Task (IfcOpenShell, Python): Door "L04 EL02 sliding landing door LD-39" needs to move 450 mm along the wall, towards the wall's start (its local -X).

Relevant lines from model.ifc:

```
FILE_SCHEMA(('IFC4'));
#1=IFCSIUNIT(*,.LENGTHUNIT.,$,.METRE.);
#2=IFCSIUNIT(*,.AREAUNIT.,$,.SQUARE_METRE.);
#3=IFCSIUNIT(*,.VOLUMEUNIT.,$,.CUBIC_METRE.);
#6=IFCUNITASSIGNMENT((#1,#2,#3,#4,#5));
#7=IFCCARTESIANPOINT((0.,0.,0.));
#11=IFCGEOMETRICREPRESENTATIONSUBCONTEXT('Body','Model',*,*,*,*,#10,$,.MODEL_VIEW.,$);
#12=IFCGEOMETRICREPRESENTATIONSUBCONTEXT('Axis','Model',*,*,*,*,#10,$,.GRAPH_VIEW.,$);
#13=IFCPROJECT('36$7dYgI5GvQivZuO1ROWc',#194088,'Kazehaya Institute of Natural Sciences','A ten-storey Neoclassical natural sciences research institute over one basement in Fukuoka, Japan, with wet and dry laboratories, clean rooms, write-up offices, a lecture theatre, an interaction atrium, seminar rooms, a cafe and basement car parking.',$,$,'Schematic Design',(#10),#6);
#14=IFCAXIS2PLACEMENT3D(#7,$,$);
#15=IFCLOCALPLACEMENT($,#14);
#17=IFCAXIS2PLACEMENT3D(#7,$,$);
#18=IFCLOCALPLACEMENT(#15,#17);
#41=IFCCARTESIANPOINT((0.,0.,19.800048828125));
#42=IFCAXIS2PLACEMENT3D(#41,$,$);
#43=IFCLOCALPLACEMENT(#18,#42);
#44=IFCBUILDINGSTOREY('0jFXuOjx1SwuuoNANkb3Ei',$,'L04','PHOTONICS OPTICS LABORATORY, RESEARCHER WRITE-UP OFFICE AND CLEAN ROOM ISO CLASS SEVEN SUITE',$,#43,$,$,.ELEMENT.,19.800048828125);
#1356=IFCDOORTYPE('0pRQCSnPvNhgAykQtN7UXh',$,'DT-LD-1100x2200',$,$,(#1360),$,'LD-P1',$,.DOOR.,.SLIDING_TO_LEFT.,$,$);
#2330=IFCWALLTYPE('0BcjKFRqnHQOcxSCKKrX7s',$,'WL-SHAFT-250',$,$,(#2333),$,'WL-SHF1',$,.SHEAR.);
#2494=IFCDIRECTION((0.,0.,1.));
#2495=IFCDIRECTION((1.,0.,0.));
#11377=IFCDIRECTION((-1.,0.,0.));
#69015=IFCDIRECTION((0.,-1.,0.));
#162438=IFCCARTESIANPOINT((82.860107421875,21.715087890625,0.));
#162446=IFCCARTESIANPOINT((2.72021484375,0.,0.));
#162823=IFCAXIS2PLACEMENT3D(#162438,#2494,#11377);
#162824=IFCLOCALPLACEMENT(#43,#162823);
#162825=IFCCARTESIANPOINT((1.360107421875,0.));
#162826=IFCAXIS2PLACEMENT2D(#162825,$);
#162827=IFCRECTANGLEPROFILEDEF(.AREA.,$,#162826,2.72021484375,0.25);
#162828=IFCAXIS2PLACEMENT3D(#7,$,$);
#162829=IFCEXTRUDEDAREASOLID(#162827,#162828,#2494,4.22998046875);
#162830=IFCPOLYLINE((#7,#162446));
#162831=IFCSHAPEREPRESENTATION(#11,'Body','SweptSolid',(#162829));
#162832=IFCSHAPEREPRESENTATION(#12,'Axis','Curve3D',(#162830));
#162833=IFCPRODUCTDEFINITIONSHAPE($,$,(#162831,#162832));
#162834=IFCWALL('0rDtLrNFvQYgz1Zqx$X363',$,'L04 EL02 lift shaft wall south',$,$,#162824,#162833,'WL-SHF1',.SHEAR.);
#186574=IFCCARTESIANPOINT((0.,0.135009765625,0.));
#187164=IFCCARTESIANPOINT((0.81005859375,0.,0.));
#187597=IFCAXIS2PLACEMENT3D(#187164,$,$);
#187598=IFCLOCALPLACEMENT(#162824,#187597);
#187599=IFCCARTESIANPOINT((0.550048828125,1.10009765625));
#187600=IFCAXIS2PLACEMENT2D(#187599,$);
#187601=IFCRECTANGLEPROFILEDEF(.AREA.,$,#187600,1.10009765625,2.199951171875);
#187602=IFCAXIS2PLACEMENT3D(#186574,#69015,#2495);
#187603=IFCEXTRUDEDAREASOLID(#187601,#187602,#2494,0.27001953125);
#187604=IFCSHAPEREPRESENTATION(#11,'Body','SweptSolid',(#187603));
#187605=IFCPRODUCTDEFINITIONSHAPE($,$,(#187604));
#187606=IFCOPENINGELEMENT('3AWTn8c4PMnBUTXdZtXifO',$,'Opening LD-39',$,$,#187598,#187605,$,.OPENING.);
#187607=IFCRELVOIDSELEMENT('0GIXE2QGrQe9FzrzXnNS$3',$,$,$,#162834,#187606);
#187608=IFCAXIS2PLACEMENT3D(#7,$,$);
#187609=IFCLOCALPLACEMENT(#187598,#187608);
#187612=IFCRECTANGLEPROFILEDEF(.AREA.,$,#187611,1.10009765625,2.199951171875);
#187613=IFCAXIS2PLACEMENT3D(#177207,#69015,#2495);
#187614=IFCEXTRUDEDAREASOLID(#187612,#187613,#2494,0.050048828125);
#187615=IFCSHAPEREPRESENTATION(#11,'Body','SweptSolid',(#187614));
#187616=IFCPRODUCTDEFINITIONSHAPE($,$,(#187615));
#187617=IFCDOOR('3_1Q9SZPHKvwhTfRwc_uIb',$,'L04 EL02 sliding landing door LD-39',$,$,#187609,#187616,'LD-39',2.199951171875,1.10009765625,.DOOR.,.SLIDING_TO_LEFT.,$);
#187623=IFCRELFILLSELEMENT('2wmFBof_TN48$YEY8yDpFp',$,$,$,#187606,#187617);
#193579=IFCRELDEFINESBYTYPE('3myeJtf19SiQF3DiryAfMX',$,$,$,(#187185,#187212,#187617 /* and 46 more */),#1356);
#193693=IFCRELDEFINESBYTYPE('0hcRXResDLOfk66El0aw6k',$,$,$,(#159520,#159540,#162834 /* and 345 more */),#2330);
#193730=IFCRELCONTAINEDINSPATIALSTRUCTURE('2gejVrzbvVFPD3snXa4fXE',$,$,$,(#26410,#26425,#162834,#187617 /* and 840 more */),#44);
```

```python
import ifcopenshell
import ifcopenshell.api.geometry
import ifcopenshell.util.placement
import ifcopenshell.util.unit

model = ifcopenshell.open("model.ifc")
unit_scale = ifcopenshell.util.unit.calculate_unit_scale(model)

door = model.by_guid("3_1Q9SZPHKvwhTfRwc_uIb")
opening = door.FillsVoids[0].RelatingOpeningElement
wall = opening.VoidsElements[0].RelatingBuildingElement

wall_matrix = ifcopenshell.util.placement.get_local_placement(wall.ObjectPlacement)
shift = wall_matrix[:3, 0] * -0.45 / unit_scale
before = ifcopenshell.util.placement.get_local_placement(door.ObjectPlacement)[:3, 3].copy()

# The door is placed relative to its opening, so it follows when the opening moves.
matrix = ifcopenshell.util.placement.get_local_placement(opening.ObjectPlacement)
matrix[:3, 3] += shift
ifcopenshell.api.geometry.edit_object_placement(
    model, product=opening, matrix=matrix, is_si=False, should_transform_children=True
)

after = ifcopenshell.util.placement.get_local_placement(door.ObjectPlacement)[:3, 3]
print("door moved by", (after - before).round(3) + 0.0)

model.write("model_updated.ifc")
```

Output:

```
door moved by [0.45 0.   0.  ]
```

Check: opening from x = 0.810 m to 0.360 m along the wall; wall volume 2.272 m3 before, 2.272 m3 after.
